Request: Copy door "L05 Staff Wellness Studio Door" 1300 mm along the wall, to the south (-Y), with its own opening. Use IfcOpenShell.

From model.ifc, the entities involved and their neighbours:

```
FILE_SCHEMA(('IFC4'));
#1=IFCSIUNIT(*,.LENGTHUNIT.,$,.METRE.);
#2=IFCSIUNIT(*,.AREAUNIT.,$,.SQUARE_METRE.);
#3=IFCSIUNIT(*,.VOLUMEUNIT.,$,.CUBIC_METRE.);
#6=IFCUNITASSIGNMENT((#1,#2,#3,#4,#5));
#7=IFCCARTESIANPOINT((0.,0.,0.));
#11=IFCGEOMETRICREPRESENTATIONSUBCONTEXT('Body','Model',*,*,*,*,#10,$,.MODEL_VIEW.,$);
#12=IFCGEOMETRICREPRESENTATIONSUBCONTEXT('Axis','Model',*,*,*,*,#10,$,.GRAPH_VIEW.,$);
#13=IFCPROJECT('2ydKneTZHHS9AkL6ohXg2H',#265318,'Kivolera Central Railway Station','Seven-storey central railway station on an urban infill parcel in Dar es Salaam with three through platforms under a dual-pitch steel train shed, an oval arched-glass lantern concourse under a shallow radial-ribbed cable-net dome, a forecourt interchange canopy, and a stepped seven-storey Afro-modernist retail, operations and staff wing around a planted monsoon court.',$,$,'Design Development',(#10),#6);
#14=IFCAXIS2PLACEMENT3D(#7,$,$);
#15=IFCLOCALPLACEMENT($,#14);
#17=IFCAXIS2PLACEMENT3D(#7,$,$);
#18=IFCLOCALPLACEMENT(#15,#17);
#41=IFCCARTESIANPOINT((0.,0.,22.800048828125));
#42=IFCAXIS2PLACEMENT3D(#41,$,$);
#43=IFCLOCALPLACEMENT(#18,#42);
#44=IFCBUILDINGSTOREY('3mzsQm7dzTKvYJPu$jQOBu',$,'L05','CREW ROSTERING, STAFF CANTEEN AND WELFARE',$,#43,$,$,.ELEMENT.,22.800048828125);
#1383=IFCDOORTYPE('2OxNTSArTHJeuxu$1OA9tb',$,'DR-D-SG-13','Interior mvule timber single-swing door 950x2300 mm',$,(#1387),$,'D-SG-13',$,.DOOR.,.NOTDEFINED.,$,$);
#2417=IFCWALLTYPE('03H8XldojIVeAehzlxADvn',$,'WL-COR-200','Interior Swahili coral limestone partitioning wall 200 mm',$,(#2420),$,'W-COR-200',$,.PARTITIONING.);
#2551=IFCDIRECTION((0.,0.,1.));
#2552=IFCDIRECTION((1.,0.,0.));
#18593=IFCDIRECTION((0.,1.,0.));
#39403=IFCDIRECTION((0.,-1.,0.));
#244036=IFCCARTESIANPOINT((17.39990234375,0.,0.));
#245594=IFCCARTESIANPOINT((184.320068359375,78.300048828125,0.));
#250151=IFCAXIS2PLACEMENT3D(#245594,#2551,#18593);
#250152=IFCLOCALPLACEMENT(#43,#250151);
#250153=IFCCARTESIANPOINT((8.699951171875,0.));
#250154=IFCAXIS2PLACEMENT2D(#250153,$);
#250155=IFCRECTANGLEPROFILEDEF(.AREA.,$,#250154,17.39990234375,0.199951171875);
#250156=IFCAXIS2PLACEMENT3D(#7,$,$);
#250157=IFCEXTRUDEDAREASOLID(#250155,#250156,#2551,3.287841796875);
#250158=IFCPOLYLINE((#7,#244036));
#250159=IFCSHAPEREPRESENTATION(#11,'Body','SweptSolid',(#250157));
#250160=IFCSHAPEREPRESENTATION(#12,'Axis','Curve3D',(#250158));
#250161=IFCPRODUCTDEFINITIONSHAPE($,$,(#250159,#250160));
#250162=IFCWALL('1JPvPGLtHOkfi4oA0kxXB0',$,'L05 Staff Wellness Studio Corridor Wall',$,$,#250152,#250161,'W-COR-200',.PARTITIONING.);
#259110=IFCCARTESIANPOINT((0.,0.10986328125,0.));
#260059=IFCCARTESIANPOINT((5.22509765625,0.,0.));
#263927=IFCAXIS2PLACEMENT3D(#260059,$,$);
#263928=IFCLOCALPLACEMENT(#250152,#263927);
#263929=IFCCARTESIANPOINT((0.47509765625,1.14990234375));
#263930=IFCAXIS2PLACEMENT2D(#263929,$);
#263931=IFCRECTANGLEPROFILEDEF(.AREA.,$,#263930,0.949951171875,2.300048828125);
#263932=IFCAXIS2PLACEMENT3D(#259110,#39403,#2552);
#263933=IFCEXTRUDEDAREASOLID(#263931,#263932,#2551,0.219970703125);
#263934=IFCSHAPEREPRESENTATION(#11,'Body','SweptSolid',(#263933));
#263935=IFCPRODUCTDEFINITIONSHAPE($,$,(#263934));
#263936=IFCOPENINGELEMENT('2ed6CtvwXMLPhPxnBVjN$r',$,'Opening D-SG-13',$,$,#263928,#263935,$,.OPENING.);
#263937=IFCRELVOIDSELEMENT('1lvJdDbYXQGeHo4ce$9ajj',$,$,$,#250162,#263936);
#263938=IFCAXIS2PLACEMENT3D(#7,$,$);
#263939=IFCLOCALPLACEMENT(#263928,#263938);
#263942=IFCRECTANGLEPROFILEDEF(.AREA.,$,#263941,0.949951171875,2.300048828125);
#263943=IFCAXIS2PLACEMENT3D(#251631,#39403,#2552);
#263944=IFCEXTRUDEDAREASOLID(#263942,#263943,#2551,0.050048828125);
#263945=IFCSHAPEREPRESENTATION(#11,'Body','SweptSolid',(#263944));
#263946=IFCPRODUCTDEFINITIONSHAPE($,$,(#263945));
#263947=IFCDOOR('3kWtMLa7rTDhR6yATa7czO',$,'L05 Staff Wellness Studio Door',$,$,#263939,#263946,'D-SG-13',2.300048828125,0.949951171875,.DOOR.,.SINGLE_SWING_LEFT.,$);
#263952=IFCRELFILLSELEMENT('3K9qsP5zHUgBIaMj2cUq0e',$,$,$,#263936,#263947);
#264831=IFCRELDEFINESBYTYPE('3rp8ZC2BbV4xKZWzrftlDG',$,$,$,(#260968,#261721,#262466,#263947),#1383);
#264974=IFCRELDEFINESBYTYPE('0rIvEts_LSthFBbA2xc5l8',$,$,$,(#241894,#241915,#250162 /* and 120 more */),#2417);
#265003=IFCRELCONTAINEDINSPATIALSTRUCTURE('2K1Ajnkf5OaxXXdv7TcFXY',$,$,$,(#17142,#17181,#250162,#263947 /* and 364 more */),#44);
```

```python
import ifcopenshell
import ifcopenshell.api.feature
import ifcopenshell.api.geometry
import ifcopenshell.api.root
import ifcopenshell.geom
import ifcopenshell.util.element
import ifcopenshell.util.placement
import ifcopenshell.util.shape

model = ifcopenshell.open("model.ifc")
settings = ifcopenshell.geom.settings()


def volume(element):
    """Net volume in cubic metres, openings subtracted."""
    shape = ifcopenshell.geom.create_shape(settings, element)
    return ifcopenshell.util.shape.get_volume(shape.geometry)


door = model.by_guid("3kWtMLa7rTDhR6yATa7czO")
opening = door.FillsVoids[0].RelatingOpeningElement
wall = opening.VoidsElements[0].RelatingBuildingElement
before = volume(wall)
shift = ifcopenshell.util.placement.get_local_placement(wall.ObjectPlacement)[:3, 0] * -1.3

# copy_class copies the void relationship, type, container and properties, but no geometry.
new_opening = ifcopenshell.api.root.copy_class(model, product=opening)
new_opening.Representation = ifcopenshell.util.element.copy_deep(
    model, opening.Representation, exclude=["IfcGeometricRepresentationContext", "IfcRepresentationMap"]
)
new_door = ifcopenshell.api.root.copy_class(model, product=door)
new_door.Representation = ifcopenshell.util.element.copy_deep(
    model, door.Representation, exclude=["IfcGeometricRepresentationContext", "IfcRepresentationMap"]
)
new_door.Tag = None
ifcopenshell.api.feature.add_filling(model, opening=new_opening, element=new_door)

for old, new in ((opening, new_opening), (door, new_door)):
    matrix = ifcopenshell.util.placement.get_local_placement(old.ObjectPlacement)
    matrix[:3, 3] += shift
    ifcopenshell.api.geometry.edit_object_placement(model, product=new, matrix=matrix, is_si=False)

after = volume(wall)

print(f"wall volume {before:.3f} -> {after:.3f} m3")

model.write("model_v2.ifc")
```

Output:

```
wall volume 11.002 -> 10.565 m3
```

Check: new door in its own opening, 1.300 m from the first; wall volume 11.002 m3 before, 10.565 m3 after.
